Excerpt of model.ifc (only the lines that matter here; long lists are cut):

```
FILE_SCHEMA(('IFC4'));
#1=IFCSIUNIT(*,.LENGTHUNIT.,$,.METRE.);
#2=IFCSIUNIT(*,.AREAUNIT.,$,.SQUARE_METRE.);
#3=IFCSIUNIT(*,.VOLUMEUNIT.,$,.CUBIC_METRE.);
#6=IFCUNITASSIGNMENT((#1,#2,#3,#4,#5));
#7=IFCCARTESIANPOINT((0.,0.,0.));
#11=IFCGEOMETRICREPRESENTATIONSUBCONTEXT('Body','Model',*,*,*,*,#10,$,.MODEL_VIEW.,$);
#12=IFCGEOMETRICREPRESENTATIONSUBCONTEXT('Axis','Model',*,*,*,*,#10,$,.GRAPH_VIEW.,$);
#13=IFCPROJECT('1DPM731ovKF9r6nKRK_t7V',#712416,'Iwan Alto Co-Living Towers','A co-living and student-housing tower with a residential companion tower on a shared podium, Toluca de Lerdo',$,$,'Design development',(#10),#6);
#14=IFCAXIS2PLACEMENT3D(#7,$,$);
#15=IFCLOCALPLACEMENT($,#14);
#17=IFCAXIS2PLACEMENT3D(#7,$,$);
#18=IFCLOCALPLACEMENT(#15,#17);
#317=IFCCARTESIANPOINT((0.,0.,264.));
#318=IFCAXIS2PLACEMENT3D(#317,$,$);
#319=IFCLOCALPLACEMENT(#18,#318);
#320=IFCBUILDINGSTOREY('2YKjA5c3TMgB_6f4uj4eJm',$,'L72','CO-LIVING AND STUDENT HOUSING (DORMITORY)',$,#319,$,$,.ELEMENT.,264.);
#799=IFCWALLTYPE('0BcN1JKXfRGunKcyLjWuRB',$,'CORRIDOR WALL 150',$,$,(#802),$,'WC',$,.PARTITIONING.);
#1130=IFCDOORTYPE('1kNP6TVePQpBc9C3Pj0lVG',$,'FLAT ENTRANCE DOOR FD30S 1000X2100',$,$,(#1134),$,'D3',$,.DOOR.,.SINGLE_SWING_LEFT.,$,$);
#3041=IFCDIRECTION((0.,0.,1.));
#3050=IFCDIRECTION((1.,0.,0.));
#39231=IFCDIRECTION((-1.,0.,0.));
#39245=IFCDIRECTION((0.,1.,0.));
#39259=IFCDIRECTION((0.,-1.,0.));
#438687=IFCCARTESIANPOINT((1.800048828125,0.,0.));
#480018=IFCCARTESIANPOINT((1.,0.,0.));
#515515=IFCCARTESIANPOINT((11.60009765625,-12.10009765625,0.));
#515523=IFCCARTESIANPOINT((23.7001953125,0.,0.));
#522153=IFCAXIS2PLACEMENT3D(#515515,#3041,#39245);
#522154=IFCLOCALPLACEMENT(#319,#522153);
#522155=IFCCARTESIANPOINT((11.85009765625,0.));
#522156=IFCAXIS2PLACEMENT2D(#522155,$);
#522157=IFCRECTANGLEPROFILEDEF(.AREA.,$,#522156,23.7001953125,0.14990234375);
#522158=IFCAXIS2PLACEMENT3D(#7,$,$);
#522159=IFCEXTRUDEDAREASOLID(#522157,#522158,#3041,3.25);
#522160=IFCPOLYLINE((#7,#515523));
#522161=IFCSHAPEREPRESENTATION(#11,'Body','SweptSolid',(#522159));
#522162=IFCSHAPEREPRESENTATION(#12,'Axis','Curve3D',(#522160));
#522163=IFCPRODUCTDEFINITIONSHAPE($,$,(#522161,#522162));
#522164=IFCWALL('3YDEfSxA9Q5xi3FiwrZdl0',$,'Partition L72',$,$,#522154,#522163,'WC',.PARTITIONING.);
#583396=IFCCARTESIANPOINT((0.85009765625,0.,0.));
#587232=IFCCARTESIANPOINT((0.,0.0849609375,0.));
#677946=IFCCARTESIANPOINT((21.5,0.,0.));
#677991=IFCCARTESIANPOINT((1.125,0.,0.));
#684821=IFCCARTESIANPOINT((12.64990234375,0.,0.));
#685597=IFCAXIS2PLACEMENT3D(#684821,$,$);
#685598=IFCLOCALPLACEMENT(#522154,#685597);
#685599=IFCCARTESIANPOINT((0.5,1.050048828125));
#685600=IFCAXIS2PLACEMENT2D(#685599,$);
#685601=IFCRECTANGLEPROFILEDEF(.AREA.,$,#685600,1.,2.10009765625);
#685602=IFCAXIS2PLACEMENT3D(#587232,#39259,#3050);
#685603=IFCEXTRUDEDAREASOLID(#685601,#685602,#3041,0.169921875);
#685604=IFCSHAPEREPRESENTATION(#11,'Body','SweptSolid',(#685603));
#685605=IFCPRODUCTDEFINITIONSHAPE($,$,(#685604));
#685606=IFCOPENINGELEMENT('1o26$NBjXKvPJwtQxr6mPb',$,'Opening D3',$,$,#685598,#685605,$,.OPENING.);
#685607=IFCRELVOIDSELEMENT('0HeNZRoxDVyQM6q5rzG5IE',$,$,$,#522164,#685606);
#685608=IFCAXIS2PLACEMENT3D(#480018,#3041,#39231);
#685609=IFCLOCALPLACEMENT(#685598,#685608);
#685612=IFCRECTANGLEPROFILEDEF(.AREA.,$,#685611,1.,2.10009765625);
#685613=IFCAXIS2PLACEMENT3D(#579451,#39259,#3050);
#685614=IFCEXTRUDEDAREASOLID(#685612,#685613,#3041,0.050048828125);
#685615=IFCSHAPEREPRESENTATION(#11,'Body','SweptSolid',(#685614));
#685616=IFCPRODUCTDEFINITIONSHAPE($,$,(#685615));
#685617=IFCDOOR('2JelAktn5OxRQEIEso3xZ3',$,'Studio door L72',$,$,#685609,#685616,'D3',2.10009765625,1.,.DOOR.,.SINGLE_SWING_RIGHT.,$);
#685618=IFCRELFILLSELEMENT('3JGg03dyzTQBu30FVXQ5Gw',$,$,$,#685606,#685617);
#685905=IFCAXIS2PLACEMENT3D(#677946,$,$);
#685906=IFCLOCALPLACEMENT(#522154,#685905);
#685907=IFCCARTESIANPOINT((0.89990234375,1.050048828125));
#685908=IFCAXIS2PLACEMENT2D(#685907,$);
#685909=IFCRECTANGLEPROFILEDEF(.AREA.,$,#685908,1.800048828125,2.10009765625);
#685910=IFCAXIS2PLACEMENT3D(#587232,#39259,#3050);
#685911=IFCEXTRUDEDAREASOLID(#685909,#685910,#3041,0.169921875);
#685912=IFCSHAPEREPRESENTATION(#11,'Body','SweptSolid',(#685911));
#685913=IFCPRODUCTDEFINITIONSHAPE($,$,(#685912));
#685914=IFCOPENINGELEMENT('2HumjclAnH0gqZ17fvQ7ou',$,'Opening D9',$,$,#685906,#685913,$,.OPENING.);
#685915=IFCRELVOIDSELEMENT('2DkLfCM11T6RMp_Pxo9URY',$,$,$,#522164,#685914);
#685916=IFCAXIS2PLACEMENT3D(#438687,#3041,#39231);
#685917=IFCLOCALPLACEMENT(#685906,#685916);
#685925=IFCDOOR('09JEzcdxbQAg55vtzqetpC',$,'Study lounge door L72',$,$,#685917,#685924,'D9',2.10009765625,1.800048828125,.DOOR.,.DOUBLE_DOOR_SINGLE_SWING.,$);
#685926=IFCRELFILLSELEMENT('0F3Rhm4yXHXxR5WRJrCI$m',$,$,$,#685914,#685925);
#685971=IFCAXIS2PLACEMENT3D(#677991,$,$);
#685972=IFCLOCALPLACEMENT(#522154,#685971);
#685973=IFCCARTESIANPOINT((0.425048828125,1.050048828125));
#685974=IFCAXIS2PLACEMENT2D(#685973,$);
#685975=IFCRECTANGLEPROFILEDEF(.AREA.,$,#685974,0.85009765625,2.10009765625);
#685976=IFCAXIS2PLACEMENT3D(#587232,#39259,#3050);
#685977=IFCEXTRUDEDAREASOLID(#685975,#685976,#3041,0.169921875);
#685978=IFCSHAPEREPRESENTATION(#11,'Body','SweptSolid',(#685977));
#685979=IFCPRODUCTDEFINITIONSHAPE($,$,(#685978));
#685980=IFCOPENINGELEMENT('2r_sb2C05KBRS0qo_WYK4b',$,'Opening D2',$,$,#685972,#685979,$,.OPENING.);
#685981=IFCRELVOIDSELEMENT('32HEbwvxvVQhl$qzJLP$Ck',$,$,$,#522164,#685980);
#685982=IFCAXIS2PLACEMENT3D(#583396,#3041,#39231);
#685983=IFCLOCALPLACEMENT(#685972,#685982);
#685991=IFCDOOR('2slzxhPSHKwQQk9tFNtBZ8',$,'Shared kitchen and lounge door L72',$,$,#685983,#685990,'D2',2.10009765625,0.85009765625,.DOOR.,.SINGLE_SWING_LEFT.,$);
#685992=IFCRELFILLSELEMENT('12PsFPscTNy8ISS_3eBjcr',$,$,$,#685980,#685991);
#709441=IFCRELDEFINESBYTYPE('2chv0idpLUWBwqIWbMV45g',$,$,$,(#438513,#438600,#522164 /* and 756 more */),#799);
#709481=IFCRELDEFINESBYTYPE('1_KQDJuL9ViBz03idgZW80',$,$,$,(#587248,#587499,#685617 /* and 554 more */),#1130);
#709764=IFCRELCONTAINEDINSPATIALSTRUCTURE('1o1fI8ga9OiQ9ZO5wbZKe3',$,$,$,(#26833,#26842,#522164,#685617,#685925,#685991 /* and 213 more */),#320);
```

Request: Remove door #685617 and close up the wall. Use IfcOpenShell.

```python
import ifcopenshell
import ifcopenshell.api.feature
import ifcopenshell.api.root
import ifcopenshell.geom
import ifcopenshell.util.shape

model = ifcopenshell.open("model.ifc")
settings = ifcopenshell.geom.settings()


def volume(element):
    """Net volume in cubic metres, openings subtracted."""
    shape = ifcopenshell.geom.create_shape(settings, element)
    return ifcopenshell.util.shape.get_volume(shape.geometry)


door = model.by_guid("2JelAktn5OxRQEIEso3xZ3")
opening = door.FillsVoids[0].RelatingOpeningElement
wall = opening.VoidsElements[0].RelatingBuildingElement
before = volume(wall)

ifcopenshell.api.root.remove_product(model, product=door)
ifcopenshell.api.feature.remove_feature(model, feature=opening)

after = volume(wall)

print(f"wall volume {before:.3f} -> {after:.3f} m3")

model.write("model_updated.ifc")
```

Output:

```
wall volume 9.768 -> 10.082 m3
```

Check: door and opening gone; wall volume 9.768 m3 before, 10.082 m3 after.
